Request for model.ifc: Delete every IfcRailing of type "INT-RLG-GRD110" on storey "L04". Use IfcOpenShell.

First a look at what the model holds.

```python
import ifcopenshell
import ifcopenshell.util.element

model = ifcopenshell.open("model.ifc")
print(model.schema)
storey = next(s for s in model.by_type("IfcBuildingStorey") if s.Name == "L04")
railings = [e for e in ifcopenshell.util.element.get_decomposition(storey) if e.is_a("IfcRailing")]
seen = {}
for e in railings:
    element_type = ifcopenshell.util.element.get_type(e)
    name = element_type.Name if element_type not in (None, e) else None
    seen[name] = seen.get(name, 0) + 1
for name, count in sorted(seen.items(), key=str):
    print(count, "x", name)
```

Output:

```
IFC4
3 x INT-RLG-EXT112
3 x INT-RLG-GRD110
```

```python
import ifcopenshell
import ifcopenshell.api.root
import ifcopenshell.util.element

model = ifcopenshell.open("model.ifc")

storey = next(s for s in model.by_type("IfcBuildingStorey") if s.Name == "L04")
railings = [e for e in ifcopenshell.util.element.get_decomposition(storey) if e.is_a("IfcRailing")]
targets = [e for e in railings if (t := ifcopenshell.util.element.get_type(e)) not in (None, e) and t.Name == "INT-RLG-GRD110"]

for e in targets:
    ifcopenshell.api.root.remove_product(model, product=e)
print(len(targets), "removed")

model.write("model_v2.ifc")
```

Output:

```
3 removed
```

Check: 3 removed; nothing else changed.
